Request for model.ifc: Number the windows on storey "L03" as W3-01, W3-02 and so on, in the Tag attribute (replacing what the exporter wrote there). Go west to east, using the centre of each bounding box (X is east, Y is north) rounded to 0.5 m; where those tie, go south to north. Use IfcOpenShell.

First a look at what the model holds.

```python
import ifcopenshell
import ifcopenshell.util.element
import ifcopenshell.util.placement

model = ifcopenshell.open("model.ifc")
print(model.schema)
storey = next(s for s in model.by_type("IfcBuildingStorey") if s.Name == "L03")
windows = [e for e in ifcopenshell.util.element.get_decomposition(storey) if e.is_a("IfcWindow")]
for e in sorted(windows, key=lambda e: e.id()):
    origin = ifcopenshell.util.placement.get_local_placement(e.ObjectPlacement)[:3, 3]
    print(e.id(), e.Tag, e.Name, origin.round(2) + 0.0, sep=" | ")
```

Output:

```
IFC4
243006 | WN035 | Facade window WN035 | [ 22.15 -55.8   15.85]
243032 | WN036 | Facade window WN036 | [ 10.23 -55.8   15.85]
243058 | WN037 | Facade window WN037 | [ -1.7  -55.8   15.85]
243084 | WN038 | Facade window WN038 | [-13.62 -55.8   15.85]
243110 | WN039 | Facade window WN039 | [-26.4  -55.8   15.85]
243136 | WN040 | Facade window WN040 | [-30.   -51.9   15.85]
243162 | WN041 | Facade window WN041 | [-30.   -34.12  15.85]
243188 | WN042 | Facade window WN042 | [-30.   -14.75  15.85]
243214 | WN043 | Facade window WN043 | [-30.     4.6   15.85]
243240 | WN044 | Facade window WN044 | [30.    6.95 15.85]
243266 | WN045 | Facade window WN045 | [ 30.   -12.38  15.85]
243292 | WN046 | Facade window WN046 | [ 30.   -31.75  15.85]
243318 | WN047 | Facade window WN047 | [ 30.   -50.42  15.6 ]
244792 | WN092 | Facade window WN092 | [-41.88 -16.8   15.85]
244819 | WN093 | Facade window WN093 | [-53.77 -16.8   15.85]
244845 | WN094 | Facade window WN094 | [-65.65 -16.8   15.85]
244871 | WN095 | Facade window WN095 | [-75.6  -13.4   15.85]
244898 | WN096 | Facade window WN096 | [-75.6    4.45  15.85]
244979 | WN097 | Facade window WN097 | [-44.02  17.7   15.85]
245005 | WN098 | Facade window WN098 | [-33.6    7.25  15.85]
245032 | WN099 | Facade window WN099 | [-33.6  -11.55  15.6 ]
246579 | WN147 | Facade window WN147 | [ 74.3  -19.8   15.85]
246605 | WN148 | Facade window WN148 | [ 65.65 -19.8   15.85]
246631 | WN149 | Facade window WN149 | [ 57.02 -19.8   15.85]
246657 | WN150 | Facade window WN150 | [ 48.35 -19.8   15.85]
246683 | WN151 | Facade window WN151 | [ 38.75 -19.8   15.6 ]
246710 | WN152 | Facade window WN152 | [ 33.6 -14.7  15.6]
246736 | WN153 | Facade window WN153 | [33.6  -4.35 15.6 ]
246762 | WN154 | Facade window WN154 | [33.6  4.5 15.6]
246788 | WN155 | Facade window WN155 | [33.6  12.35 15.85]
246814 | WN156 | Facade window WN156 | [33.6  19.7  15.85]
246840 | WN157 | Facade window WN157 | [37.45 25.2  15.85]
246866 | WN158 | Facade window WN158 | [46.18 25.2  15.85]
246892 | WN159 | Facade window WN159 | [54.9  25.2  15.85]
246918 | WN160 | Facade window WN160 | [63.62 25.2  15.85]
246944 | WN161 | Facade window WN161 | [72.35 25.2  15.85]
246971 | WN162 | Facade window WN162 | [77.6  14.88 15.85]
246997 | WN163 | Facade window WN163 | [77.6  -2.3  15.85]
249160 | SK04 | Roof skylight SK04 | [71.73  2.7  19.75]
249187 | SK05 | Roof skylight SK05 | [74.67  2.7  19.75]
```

```python
import ifcopenshell
import ifcopenshell.geom
import ifcopenshell.util.element
import ifcopenshell.util.shape

model = ifcopenshell.open("model.ifc")
settings = ifcopenshell.geom.settings()
settings.set("use-world-coords", True)


def centre(element):
    shape = ifcopenshell.geom.create_shape(settings, element)
    return ifcopenshell.util.shape.get_bbox_centroid(shape.geometry)


storey = next(s for s in model.by_type("IfcBuildingStorey") if s.Name == "L03")
windows = [e for e in ifcopenshell.util.element.get_decomposition(storey) if e.is_a("IfcWindow")]

# Insertion points can sit at a corner or the storey origin, so sort by the geometry (in metres).
centres = {e: centre(e) for e in windows}
windows.sort(key=lambda e: (round(centres[e][0] / 0.5), centres[e][1]))

for i, e in enumerate(windows, start=1):
    number = f"W3-{i:02d}"
    e.Tag = number
    print(e.id(), number)

model.write("model-out.ifc")
```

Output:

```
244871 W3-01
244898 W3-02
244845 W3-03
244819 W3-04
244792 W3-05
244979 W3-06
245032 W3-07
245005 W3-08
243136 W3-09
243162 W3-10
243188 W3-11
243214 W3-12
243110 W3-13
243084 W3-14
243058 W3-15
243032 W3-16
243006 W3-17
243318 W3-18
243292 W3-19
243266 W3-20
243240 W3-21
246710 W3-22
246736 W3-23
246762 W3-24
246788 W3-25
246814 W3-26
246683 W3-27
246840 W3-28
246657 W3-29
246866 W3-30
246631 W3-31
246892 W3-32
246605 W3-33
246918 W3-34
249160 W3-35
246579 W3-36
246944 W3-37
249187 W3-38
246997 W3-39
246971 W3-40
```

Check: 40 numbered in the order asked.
